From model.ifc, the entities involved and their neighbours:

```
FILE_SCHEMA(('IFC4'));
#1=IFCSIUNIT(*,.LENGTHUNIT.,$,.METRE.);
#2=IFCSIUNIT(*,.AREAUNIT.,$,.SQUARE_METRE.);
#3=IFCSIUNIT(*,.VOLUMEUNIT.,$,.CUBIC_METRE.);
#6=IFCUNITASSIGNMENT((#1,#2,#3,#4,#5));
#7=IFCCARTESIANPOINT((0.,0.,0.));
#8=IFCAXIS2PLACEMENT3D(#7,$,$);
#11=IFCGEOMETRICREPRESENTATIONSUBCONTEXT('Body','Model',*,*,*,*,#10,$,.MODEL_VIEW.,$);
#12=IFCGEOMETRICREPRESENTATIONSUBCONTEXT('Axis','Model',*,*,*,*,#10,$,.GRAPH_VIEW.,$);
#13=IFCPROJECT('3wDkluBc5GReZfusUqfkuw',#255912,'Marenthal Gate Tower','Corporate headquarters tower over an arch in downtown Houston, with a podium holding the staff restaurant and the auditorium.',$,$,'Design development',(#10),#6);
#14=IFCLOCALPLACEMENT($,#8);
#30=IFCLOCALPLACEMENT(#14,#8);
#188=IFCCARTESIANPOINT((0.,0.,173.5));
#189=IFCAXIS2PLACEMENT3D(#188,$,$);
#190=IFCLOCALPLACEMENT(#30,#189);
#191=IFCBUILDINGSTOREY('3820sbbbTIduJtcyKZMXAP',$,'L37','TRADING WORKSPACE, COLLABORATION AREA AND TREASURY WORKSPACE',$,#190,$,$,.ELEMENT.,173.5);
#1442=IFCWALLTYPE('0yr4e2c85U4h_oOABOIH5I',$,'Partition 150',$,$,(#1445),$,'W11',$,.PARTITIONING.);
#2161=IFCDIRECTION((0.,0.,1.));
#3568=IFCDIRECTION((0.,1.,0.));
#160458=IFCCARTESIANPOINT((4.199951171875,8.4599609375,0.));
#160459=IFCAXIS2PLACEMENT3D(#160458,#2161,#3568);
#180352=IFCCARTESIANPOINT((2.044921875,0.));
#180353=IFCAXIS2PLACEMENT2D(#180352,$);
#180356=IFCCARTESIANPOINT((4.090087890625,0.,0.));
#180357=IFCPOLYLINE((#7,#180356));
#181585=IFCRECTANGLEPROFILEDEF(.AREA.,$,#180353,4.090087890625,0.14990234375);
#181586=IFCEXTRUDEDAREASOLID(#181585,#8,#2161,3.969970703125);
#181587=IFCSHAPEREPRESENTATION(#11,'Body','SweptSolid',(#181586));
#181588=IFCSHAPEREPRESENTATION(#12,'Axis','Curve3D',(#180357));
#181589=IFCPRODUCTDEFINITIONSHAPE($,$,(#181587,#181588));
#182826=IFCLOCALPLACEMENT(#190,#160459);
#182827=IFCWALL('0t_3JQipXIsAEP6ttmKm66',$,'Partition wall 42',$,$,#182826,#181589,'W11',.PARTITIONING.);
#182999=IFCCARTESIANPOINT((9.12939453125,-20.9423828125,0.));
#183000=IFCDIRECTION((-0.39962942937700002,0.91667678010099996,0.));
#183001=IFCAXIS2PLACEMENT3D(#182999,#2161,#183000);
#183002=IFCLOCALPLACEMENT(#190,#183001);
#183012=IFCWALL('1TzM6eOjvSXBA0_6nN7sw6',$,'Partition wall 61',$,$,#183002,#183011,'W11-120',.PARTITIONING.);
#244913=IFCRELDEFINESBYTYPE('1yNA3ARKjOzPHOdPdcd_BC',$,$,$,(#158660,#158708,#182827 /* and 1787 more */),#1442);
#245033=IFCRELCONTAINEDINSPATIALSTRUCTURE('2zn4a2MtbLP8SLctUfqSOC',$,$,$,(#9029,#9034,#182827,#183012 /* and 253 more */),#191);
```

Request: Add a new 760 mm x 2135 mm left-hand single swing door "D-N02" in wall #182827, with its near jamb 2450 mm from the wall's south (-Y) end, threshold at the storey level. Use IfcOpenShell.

```python
import numpy as np
import ifcopenshell
import ifcopenshell.api.feature
import ifcopenshell.api.geometry
import ifcopenshell.api.root
import ifcopenshell.api.spatial
import ifcopenshell.geom
import ifcopenshell.util.element
import ifcopenshell.util.placement
import ifcopenshell.util.representation
import ifcopenshell.util.shape
import ifcopenshell.util.unit

model = ifcopenshell.open("model.ifc")
unit_scale = ifcopenshell.util.unit.calculate_unit_scale(model)
settings = ifcopenshell.geom.settings()


def volume(element):
    """Net volume in cubic metres, openings subtracted."""
    shape = ifcopenshell.geom.create_shape(settings, element)
    return ifcopenshell.util.shape.get_volume(shape.geometry)


wall = model.by_guid("0t_3JQipXIsAEP6ttmKm66")
storey = ifcopenshell.util.element.get_container(wall, ifc_class="IfcBuildingStorey")
context = ifcopenshell.util.representation.get_context(model, "Model", "Body", "MODEL_VIEW")
before = volume(wall)

width, height, from_end, sill = 0.76, 2.135, 2.45, 0.0  # metres

# The wall runs along its own X axis, and the end named is its -X end.
wall_shape = ifcopenshell.geom.create_shape(settings, wall)
x, y, z = ifcopenshell.util.shape.get_vertices(wall_shape.geometry).T
start = x.min() + from_end
face, thickness = float(y.min()), float(y.max() - y.min())
wall_matrix = ifcopenshell.util.placement.get_local_placement(wall.ObjectPlacement)
level = ifcopenshell.util.placement.get_local_placement(storey.ObjectPlacement)[2, 3]


def in_wall(x, y):
    """Placement at x, y metres in the wall's axes, at sill height."""
    matrix = wall_matrix.copy()
    matrix[:, 3] = wall_matrix @ np.array([x / unit_scale, y / unit_scale, 0.0, 1.0])
    matrix[2, 3] = level + sill / unit_scale
    return matrix


# Opening: a box that overshoots both wall faces by 50 mm.
opening = ifcopenshell.api.root.create_entity(model, ifc_class="IfcOpeningElement", predefined_type="OPENING")
box = ifcopenshell.api.geometry.add_wall_representation(
    model, context=context, length=width, height=height, thickness=thickness + 0.1
)
ifcopenshell.api.geometry.assign_representation(model, product=opening, representation=box)
ifcopenshell.api.geometry.edit_object_placement(model, product=opening, matrix=in_wall(start, face - 0.05), is_si=False)
ifcopenshell.api.feature.add_feature(model, feature=opening, element=wall)

door = ifcopenshell.api.root.create_entity(model, ifc_class="IfcDoor", name="D-N02", predefined_type="DOOR")
door.OverallWidth, door.OverallHeight = width / unit_scale, height / unit_scale
door.OperationType = "SINGLE_SWING_LEFT"
body = ifcopenshell.api.geometry.add_door_representation(
    model,
    context=context,
    overall_width=door.OverallWidth,
    overall_height=door.OverallHeight,
    operation_type="SINGLE_SWING_LEFT",
    lining_properties={"LiningDepth": thickness / unit_scale, "ThresholdDepth": thickness / unit_scale},
)
ifcopenshell.api.geometry.assign_representation(model, product=door, representation=body)
ifcopenshell.api.spatial.assign_container(model, products=[door], relating_structure=storey)
ifcopenshell.api.feature.add_filling(model, opening=opening, element=door)

# The lining spans the wall, so the door starts at the wall face.
ifcopenshell.api.geometry.edit_object_placement(model, product=door, matrix=in_wall(start, face), is_si=False)

after = volume(wall)

print(f"wall volume {before:.3f} -> {after:.3f} m3")

model.write("model_updated.ifc")
```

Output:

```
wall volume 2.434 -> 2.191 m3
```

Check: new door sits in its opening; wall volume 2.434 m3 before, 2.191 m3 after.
